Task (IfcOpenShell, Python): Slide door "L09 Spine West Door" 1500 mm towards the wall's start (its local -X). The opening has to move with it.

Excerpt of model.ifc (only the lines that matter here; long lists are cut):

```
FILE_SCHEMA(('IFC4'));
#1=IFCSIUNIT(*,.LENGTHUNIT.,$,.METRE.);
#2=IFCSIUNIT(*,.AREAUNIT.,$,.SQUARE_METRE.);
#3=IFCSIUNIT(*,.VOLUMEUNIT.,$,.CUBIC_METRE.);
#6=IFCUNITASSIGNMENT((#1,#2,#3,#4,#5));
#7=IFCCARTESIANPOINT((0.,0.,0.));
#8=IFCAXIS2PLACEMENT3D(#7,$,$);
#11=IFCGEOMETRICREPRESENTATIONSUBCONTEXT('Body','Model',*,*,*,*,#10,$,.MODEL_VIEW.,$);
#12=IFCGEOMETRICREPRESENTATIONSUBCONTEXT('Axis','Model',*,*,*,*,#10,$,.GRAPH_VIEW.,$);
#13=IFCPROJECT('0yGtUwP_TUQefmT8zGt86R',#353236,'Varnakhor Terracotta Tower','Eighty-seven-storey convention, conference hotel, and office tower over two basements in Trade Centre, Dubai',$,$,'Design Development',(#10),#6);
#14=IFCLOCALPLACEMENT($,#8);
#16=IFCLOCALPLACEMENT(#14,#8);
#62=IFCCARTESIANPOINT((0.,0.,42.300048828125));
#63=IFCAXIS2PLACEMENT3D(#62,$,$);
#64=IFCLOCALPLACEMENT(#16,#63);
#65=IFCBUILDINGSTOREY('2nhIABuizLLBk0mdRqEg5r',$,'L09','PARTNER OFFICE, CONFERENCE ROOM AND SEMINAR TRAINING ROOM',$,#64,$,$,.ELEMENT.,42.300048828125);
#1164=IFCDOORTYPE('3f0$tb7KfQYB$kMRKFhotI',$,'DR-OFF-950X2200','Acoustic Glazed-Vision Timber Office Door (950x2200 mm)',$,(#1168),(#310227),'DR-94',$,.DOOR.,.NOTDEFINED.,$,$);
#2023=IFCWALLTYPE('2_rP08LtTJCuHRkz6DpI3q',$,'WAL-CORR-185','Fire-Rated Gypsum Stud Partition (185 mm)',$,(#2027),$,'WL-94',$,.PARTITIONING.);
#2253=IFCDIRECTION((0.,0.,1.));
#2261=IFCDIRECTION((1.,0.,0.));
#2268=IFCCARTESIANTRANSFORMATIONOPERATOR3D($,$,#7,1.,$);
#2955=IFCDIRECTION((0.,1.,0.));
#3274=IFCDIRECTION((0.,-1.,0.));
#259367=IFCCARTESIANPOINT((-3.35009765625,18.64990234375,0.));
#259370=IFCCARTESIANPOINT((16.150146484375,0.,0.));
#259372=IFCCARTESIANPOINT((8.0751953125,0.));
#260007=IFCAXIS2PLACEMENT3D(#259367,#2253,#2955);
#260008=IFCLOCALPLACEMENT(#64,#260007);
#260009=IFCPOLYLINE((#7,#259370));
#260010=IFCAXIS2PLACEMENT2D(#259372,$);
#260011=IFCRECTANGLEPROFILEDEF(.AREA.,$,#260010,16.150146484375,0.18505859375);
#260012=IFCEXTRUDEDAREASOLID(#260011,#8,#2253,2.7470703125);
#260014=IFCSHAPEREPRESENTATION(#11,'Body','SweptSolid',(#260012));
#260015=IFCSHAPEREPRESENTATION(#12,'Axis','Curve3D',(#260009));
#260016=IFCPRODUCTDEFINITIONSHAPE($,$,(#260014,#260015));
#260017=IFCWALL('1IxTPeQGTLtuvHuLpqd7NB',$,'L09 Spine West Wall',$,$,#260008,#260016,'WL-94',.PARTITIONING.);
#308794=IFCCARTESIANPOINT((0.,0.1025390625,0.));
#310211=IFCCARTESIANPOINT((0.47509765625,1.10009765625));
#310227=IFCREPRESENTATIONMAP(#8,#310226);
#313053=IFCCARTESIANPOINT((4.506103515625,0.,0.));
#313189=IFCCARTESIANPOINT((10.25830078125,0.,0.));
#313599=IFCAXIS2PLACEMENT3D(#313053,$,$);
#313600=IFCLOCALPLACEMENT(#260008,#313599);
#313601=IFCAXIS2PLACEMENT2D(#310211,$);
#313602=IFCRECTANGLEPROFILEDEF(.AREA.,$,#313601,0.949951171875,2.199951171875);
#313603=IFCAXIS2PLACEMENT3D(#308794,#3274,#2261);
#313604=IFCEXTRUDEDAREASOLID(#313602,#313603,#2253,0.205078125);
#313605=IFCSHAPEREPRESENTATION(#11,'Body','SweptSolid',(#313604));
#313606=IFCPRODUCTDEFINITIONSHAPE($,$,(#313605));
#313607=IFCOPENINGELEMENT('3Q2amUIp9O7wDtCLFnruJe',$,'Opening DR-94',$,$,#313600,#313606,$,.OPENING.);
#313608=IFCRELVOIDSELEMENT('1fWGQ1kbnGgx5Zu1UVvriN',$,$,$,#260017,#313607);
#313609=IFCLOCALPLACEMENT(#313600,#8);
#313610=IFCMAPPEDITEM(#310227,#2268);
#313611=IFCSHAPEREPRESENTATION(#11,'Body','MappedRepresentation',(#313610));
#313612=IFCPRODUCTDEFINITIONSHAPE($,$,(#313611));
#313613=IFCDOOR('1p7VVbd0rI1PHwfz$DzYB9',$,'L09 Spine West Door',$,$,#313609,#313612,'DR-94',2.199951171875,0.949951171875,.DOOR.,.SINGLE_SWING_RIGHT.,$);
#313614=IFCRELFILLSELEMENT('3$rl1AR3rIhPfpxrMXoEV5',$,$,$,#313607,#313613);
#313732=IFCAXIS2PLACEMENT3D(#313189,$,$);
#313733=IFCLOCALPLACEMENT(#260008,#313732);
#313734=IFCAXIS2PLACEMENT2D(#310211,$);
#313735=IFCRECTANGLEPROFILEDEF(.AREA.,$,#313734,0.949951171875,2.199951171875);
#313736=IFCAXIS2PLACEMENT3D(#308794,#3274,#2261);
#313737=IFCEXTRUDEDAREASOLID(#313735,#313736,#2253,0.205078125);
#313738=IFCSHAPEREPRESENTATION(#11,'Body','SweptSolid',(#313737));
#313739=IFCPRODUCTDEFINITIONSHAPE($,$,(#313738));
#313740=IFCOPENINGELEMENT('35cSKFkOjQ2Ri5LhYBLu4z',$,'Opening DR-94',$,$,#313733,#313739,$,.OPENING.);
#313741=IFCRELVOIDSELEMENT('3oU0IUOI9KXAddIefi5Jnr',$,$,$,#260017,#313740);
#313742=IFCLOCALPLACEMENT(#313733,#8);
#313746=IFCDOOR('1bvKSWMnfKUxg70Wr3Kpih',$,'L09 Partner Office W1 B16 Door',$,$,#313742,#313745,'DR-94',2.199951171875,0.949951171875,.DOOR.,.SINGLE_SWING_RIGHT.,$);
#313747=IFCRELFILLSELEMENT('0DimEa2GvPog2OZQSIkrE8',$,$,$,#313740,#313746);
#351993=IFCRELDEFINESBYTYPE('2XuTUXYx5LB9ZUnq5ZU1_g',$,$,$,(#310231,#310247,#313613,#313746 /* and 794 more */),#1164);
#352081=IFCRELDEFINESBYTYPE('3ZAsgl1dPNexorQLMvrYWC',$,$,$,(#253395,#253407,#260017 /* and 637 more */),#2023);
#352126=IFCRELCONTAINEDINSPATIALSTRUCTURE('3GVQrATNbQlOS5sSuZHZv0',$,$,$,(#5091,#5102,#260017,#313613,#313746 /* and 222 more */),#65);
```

```python
import ifcopenshell
import ifcopenshell.api.geometry
import ifcopenshell.util.placement

model = ifcopenshell.open("model.ifc")

door = model.by_guid("1p7VVbd0rI1PHwfz$DzYB9")
opening = door.FillsVoids[0].RelatingOpeningElement
wall = opening.VoidsElements[0].RelatingBuildingElement

wall_matrix = ifcopenshell.util.placement.get_local_placement(wall.ObjectPlacement)
shift = wall_matrix[:3, 0] * -1.5
before = ifcopenshell.util.placement.get_local_placement(door.ObjectPlacement)[:3, 3].copy()

# The door is placed relative to its opening, so it follows when the opening moves.
matrix = ifcopenshell.util.placement.get_local_placement(opening.ObjectPlacement)
matrix[:3, 3] += shift
ifcopenshell.api.geometry.edit_object_placement(
    model, product=opening, matrix=matrix, is_si=False, should_transform_children=True
)

after = ifcopenshell.util.placement.get_local_placement(door.ObjectPlacement)[:3, 3]
print("door moved by", (after - before).round(3) + 0.0)

model.write("model_updated.ifc")
```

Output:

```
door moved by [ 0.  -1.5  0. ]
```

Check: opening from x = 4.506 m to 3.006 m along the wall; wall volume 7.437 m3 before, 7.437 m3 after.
